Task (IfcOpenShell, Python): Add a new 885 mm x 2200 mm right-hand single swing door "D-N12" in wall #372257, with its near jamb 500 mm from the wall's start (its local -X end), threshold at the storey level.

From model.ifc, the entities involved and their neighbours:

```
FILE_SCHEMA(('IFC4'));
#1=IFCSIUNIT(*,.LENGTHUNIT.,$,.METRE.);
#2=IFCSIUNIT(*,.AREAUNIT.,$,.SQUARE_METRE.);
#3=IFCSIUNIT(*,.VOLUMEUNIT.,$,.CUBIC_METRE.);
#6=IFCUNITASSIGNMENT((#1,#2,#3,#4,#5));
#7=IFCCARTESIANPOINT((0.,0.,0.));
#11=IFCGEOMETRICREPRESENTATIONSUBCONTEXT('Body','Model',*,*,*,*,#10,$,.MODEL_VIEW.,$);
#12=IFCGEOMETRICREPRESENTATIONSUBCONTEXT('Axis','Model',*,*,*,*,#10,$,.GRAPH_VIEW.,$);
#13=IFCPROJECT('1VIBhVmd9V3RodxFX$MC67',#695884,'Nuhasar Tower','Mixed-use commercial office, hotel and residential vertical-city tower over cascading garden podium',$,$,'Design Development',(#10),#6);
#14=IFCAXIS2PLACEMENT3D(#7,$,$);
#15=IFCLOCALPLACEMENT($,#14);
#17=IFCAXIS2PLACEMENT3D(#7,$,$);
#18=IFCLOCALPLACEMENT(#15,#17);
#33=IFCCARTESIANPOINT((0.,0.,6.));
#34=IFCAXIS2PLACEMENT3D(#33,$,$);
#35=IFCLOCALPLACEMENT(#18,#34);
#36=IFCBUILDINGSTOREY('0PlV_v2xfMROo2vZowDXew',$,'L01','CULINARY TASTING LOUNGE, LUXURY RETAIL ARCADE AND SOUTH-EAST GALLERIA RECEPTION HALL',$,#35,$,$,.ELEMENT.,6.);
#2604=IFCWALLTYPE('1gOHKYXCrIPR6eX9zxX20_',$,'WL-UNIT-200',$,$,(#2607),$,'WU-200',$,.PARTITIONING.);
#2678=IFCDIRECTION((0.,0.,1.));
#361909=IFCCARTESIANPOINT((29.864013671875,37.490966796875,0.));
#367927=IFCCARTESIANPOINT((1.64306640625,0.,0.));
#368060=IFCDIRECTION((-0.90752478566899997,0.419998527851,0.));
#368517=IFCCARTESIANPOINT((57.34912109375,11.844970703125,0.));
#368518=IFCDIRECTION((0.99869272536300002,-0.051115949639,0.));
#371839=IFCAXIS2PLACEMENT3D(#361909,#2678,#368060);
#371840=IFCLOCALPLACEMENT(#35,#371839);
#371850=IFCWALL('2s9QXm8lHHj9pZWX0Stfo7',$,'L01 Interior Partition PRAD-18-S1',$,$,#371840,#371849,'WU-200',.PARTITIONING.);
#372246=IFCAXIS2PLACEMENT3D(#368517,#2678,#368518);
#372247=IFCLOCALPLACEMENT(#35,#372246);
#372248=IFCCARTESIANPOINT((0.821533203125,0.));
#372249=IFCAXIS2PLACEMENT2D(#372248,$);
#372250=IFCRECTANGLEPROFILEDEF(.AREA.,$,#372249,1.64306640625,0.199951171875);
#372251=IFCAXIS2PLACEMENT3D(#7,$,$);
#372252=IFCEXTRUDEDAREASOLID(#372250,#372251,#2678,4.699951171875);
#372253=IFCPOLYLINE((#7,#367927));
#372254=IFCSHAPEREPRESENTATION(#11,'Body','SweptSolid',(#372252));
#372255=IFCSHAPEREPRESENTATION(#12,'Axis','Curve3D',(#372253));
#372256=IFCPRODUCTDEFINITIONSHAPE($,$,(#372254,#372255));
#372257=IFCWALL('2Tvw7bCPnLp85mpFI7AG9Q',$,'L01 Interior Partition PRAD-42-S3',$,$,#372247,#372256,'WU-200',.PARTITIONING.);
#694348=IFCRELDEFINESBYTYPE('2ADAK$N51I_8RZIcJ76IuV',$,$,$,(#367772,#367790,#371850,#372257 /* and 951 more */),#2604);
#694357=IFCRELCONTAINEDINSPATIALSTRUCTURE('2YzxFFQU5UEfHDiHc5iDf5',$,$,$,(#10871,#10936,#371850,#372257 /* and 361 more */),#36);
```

```python
import numpy as np
import ifcopenshell
import ifcopenshell.api.feature
import ifcopenshell.api.geometry
import ifcopenshell.api.root
import ifcopenshell.api.spatial
import ifcopenshell.geom
import ifcopenshell.util.element
import ifcopenshell.util.placement
import ifcopenshell.util.representation
import ifcopenshell.util.shape
import ifcopenshell.util.unit

model = ifcopenshell.open("model.ifc")
unit_scale = ifcopenshell.util.unit.calculate_unit_scale(model)
settings = ifcopenshell.geom.settings()


def volume(element):
    """Net volume in cubic metres, openings subtracted."""
    shape = ifcopenshell.geom.create_shape(settings, element)
    return ifcopenshell.util.shape.get_volume(shape.geometry)


wall = model.by_guid("2Tvw7bCPnLp85mpFI7AG9Q")
storey = ifcopenshell.util.element.get_container(wall, ifc_class="IfcBuildingStorey")
context = ifcopenshell.util.representation.get_context(model, "Model", "Body", "MODEL_VIEW")
before = volume(wall)

width, height, from_end, sill = 0.885, 2.2, 0.5, 0.0  # metres

# The wall runs along its own X axis, and the end named is its -X end.
wall_shape = ifcopenshell.geom.create_shape(settings, wall)
x, y, z = ifcopenshell.util.shape.get_vertices(wall_shape.geometry).T
start = x.min() + from_end
face, thickness = float(y.min()), float(y.max() - y.min())
wall_matrix = ifcopenshell.util.placement.get_local_placement(wall.ObjectPlacement)
level = ifcopenshell.util.placement.get_local_placement(storey.ObjectPlacement)[2, 3]


def in_wall(x, y):
    """Placement at x, y metres in the wall's axes, at sill height."""
    matrix = wall_matrix.copy()
    matrix[:, 3] = wall_matrix @ np.array([x / unit_scale, y / unit_scale, 0.0, 1.0])
    matrix[2, 3] = level + sill / unit_scale
    return matrix


# Opening: a box that overshoots both wall faces by 50 mm.
opening = ifcopenshell.api.root.create_entity(model, ifc_class="IfcOpeningElement", predefined_type="OPENING")
box = ifcopenshell.api.geometry.add_wall_representation(
    model, context=context, length=width, height=height, thickness=thickness + 0.1
)
ifcopenshell.api.geometry.assign_representation(model, product=opening, representation=box)
ifcopenshell.api.geometry.edit_object_placement(model, product=opening, matrix=in_wall(start, face - 0.05), is_si=False)
ifcopenshell.api.feature.add_feature(model, feature=opening, element=wall)

door = ifcopenshell.api.root.create_entity(model, ifc_class="IfcDoor", name="D-N12", predefined_type="DOOR")
door.OverallWidth, door.OverallHeight = width / unit_scale, height / unit_scale
door.OperationType = "SINGLE_SWING_RIGHT"
body = ifcopenshell.api.geometry.add_door_representation(
    model,
    context=context,
    overall_width=door.OverallWidth,
    overall_height=door.OverallHeight,
    operation_type="SINGLE_SWING_RIGHT",
    lining_properties={"LiningDepth": thickness / unit_scale, "ThresholdDepth": thickness / unit_scale},
)
ifcopenshell.api.geometry.assign_representation(model, product=door, representation=body)
ifcopenshell.api.spatial.assign_container(model, products=[door], relating_structure=storey)
ifcopenshell.api.feature.add_filling(model, opening=opening, element=door)

# The lining spans the wall, so the door starts at the wall face.
ifcopenshell.api.geometry.edit_object_placement(model, product=door, matrix=in_wall(start, face), is_si=False)

after = volume(wall)

print(f"wall volume {before:.3f} -> {after:.3f} m3")

model.write("model_rev.ifc")
```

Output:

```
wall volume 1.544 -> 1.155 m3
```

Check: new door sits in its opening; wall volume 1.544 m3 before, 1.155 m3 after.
